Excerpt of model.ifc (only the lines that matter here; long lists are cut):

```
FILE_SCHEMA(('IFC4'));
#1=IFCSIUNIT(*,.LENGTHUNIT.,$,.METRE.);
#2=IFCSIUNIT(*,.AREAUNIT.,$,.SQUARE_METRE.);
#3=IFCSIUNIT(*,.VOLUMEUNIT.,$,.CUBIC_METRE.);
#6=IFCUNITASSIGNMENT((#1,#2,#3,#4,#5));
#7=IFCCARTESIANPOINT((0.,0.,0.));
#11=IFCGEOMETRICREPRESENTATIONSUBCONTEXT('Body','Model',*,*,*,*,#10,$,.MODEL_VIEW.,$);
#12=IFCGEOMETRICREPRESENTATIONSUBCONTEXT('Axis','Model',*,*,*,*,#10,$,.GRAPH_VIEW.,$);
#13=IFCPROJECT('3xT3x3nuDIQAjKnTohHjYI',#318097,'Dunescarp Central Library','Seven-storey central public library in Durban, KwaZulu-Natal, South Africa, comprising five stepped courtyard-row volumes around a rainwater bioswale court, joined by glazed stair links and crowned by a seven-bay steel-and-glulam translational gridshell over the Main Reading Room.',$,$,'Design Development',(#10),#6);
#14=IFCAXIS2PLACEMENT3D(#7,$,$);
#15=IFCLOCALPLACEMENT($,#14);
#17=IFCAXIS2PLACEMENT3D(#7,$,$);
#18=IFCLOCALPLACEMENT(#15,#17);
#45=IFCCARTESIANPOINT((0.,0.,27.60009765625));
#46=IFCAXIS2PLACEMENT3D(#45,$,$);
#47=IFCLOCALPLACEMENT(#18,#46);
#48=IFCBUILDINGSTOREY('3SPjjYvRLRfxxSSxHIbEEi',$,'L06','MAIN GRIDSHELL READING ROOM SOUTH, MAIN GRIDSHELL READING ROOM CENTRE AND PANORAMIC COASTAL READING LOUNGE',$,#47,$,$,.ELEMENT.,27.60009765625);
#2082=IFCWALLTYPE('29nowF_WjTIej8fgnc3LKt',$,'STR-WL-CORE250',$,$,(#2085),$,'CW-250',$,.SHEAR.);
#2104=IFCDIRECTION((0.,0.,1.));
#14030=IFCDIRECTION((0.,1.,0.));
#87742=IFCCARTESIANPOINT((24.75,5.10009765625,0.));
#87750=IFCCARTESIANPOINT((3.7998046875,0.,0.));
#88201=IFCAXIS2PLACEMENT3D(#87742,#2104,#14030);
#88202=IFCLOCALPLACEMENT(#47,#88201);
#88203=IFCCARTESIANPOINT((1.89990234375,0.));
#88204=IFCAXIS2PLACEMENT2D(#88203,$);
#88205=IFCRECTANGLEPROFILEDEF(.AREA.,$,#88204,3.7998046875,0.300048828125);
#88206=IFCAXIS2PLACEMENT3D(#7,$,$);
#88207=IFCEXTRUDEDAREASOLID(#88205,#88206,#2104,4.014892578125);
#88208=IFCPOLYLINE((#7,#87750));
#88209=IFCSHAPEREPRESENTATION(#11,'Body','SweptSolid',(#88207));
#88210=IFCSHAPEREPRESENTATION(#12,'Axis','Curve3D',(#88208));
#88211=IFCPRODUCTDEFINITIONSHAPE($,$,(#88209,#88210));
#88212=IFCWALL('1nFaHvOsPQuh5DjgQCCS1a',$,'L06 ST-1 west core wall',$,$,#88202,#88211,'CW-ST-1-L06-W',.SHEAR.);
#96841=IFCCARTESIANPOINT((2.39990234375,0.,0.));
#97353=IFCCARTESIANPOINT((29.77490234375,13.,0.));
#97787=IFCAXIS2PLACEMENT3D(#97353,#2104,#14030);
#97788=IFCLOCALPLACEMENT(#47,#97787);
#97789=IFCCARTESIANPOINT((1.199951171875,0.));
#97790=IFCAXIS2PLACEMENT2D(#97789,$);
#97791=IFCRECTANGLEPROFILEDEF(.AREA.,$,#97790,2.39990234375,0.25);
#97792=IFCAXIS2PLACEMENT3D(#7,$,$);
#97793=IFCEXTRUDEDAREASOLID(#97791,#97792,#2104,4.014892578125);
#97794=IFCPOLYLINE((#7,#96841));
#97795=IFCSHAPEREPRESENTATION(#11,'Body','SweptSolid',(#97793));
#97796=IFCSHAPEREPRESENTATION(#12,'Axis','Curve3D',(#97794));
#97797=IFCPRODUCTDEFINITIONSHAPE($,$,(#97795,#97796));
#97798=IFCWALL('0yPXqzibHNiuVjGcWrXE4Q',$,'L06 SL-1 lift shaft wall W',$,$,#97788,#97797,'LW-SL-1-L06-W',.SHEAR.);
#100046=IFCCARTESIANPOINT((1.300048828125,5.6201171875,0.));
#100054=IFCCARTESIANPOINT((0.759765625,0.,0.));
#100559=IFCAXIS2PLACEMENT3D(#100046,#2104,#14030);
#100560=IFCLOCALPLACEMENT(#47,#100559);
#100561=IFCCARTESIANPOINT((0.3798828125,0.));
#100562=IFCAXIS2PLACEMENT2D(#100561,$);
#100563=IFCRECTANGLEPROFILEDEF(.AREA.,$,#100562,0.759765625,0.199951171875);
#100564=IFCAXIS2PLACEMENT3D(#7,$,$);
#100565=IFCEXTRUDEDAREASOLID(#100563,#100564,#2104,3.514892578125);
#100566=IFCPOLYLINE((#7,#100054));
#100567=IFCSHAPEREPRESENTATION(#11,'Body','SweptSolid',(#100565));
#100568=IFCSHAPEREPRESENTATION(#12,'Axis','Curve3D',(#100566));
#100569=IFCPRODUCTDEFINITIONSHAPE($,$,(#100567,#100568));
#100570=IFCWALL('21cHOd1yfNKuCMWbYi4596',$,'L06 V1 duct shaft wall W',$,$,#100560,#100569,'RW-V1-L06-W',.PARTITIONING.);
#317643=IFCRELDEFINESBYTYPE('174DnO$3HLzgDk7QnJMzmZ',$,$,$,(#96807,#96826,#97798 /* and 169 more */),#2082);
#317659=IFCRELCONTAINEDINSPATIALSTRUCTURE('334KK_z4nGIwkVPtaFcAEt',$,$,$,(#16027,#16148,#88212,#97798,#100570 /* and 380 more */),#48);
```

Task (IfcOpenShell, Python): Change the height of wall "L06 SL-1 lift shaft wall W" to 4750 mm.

```python
import ifcopenshell
import ifcopenshell.geom
import ifcopenshell.util.representation
import ifcopenshell.util.shape

model = ifcopenshell.open("model.ifc")
settings = ifcopenshell.geom.settings()


def volume(element):
    """Net volume in cubic metres, openings subtracted."""
    shape = ifcopenshell.geom.create_shape(settings, element)
    return ifcopenshell.util.shape.get_volume(shape.geometry)


wall = model.by_id(97798)
before = volume(wall)

body = ifcopenshell.util.representation.get_representation(wall, "Model", "Body")
solid = body.Items[0]
old_height = solid.Depth
solid.Depth = 4.75
after = volume(wall)

print(f"height {old_height:g} -> {solid.Depth:g}, volume {before:.3f} -> {after:.3f} m3")

model.write("model-out.ifc")
```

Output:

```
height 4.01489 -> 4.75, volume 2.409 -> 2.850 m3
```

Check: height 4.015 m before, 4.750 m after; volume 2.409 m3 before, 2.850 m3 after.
